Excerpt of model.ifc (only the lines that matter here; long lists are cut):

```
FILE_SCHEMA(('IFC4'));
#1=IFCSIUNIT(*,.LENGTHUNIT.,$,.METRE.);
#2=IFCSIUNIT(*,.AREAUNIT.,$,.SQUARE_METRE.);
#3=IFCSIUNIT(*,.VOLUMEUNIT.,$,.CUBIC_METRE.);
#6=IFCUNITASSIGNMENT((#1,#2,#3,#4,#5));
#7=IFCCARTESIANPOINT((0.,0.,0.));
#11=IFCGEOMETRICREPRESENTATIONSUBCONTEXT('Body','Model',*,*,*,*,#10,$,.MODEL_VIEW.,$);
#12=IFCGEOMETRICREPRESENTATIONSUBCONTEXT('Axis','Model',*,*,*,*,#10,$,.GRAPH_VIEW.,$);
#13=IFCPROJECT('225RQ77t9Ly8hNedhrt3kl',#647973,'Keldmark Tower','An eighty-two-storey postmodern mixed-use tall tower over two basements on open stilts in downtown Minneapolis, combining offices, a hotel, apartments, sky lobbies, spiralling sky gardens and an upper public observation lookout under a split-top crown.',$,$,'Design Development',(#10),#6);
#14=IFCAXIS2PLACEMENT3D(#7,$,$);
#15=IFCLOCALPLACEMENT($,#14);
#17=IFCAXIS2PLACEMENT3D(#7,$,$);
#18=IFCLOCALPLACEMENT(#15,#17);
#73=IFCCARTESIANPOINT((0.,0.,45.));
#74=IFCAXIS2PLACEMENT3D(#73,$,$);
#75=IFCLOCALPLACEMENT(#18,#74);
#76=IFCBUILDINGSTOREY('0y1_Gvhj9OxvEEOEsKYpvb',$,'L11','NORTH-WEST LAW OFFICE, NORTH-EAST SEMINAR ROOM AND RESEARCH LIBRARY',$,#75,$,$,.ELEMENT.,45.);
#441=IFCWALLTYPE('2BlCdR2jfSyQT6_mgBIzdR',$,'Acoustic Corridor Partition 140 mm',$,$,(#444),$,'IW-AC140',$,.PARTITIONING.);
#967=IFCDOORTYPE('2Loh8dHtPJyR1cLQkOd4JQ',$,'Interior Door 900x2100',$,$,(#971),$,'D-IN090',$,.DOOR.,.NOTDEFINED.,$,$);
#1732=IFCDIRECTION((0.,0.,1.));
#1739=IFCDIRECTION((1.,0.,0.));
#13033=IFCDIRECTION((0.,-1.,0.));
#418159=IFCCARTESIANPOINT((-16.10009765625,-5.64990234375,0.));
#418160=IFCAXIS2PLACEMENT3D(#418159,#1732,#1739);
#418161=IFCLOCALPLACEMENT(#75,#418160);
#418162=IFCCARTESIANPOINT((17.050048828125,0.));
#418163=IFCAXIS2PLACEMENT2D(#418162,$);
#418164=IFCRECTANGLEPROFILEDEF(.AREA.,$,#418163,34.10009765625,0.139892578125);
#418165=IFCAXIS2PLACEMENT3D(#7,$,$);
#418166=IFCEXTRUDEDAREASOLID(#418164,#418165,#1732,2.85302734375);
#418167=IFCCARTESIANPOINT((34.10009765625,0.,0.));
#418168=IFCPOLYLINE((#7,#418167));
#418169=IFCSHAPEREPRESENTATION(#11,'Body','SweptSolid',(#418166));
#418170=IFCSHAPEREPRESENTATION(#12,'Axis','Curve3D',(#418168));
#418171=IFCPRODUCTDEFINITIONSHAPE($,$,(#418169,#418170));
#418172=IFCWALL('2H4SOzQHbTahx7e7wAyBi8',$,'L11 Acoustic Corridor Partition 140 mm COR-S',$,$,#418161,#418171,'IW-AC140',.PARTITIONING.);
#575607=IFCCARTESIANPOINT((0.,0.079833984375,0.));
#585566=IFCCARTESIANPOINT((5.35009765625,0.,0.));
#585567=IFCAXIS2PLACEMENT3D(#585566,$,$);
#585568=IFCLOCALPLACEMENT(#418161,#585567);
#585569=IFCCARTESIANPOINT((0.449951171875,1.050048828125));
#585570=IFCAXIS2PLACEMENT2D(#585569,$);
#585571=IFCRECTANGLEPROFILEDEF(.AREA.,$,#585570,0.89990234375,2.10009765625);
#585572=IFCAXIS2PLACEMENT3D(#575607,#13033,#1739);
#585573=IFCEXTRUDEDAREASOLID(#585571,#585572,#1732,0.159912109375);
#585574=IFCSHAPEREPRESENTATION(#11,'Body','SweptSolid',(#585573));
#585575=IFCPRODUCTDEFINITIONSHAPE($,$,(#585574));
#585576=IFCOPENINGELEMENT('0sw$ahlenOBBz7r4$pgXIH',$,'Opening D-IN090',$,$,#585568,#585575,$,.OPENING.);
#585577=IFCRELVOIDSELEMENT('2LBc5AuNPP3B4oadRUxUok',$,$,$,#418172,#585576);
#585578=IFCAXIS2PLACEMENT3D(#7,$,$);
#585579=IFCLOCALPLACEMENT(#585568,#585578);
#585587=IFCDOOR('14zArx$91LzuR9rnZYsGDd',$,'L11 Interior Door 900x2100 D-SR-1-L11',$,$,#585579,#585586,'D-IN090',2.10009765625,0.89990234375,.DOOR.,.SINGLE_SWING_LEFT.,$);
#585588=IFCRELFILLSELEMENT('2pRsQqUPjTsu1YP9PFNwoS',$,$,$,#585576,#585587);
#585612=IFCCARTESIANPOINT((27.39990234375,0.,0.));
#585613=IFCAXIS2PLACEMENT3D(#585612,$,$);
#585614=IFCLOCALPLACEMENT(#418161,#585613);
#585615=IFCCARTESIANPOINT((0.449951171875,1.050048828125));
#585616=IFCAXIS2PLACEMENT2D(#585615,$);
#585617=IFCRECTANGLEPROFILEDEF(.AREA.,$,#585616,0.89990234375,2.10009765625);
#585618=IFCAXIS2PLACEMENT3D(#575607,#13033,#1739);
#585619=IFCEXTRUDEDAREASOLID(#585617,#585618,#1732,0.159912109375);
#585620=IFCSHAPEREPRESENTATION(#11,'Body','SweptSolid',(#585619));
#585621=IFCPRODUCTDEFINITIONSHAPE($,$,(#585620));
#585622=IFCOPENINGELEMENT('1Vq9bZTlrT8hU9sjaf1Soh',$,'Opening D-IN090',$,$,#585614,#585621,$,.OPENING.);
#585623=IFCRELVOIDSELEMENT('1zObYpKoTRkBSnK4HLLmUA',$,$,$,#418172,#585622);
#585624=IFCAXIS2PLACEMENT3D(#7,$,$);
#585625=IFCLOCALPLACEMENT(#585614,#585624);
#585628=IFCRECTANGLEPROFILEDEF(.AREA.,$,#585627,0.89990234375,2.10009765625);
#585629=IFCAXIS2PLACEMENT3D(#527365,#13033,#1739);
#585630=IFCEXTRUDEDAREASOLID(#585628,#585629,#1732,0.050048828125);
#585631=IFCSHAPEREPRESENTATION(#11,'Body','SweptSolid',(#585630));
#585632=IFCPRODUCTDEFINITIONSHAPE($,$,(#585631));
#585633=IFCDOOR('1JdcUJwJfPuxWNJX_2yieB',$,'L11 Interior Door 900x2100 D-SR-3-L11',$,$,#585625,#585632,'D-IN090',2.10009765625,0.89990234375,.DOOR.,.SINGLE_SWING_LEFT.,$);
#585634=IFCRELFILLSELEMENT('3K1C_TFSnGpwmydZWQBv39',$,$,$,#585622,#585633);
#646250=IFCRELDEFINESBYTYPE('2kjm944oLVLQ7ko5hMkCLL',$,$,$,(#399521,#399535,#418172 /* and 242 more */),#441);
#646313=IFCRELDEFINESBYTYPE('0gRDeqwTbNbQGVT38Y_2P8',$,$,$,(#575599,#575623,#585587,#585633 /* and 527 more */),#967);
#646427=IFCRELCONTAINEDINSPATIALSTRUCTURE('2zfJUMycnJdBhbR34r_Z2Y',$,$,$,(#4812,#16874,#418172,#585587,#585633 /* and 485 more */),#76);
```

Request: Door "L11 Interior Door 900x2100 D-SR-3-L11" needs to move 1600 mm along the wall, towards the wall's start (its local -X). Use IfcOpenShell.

```python
import ifcopenshell
import ifcopenshell.api.geometry
import ifcopenshell.util.placement

model = ifcopenshell.open("model.ifc")

door = model.by_guid("1JdcUJwJfPuxWNJX_2yieB")
opening = door.FillsVoids[0].RelatingOpeningElement
wall = opening.VoidsElements[0].RelatingBuildingElement

wall_matrix = ifcopenshell.util.placement.get_local_placement(wall.ObjectPlacement)
shift = wall_matrix[:3, 0] * -1.6
before = ifcopenshell.util.placement.get_local_placement(door.ObjectPlacement)[:3, 3].copy()

# The door is placed relative to its opening, so it follows when the opening moves.
matrix = ifcopenshell.util.placement.get_local_placement(opening.ObjectPlacement)
matrix[:3, 3] += shift
ifcopenshell.api.geometry.edit_object_placement(
    model, product=opening, matrix=matrix, is_si=False, should_transform_children=True
)

after = ifcopenshell.util.placement.get_local_placement(door.ObjectPlacement)[:3, 3]
print("door moved by", (after - before).round(3) + 0.0)

model.write("model_v2.ifc")
```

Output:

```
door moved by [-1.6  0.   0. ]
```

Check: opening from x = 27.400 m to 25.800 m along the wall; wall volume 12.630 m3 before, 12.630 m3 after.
